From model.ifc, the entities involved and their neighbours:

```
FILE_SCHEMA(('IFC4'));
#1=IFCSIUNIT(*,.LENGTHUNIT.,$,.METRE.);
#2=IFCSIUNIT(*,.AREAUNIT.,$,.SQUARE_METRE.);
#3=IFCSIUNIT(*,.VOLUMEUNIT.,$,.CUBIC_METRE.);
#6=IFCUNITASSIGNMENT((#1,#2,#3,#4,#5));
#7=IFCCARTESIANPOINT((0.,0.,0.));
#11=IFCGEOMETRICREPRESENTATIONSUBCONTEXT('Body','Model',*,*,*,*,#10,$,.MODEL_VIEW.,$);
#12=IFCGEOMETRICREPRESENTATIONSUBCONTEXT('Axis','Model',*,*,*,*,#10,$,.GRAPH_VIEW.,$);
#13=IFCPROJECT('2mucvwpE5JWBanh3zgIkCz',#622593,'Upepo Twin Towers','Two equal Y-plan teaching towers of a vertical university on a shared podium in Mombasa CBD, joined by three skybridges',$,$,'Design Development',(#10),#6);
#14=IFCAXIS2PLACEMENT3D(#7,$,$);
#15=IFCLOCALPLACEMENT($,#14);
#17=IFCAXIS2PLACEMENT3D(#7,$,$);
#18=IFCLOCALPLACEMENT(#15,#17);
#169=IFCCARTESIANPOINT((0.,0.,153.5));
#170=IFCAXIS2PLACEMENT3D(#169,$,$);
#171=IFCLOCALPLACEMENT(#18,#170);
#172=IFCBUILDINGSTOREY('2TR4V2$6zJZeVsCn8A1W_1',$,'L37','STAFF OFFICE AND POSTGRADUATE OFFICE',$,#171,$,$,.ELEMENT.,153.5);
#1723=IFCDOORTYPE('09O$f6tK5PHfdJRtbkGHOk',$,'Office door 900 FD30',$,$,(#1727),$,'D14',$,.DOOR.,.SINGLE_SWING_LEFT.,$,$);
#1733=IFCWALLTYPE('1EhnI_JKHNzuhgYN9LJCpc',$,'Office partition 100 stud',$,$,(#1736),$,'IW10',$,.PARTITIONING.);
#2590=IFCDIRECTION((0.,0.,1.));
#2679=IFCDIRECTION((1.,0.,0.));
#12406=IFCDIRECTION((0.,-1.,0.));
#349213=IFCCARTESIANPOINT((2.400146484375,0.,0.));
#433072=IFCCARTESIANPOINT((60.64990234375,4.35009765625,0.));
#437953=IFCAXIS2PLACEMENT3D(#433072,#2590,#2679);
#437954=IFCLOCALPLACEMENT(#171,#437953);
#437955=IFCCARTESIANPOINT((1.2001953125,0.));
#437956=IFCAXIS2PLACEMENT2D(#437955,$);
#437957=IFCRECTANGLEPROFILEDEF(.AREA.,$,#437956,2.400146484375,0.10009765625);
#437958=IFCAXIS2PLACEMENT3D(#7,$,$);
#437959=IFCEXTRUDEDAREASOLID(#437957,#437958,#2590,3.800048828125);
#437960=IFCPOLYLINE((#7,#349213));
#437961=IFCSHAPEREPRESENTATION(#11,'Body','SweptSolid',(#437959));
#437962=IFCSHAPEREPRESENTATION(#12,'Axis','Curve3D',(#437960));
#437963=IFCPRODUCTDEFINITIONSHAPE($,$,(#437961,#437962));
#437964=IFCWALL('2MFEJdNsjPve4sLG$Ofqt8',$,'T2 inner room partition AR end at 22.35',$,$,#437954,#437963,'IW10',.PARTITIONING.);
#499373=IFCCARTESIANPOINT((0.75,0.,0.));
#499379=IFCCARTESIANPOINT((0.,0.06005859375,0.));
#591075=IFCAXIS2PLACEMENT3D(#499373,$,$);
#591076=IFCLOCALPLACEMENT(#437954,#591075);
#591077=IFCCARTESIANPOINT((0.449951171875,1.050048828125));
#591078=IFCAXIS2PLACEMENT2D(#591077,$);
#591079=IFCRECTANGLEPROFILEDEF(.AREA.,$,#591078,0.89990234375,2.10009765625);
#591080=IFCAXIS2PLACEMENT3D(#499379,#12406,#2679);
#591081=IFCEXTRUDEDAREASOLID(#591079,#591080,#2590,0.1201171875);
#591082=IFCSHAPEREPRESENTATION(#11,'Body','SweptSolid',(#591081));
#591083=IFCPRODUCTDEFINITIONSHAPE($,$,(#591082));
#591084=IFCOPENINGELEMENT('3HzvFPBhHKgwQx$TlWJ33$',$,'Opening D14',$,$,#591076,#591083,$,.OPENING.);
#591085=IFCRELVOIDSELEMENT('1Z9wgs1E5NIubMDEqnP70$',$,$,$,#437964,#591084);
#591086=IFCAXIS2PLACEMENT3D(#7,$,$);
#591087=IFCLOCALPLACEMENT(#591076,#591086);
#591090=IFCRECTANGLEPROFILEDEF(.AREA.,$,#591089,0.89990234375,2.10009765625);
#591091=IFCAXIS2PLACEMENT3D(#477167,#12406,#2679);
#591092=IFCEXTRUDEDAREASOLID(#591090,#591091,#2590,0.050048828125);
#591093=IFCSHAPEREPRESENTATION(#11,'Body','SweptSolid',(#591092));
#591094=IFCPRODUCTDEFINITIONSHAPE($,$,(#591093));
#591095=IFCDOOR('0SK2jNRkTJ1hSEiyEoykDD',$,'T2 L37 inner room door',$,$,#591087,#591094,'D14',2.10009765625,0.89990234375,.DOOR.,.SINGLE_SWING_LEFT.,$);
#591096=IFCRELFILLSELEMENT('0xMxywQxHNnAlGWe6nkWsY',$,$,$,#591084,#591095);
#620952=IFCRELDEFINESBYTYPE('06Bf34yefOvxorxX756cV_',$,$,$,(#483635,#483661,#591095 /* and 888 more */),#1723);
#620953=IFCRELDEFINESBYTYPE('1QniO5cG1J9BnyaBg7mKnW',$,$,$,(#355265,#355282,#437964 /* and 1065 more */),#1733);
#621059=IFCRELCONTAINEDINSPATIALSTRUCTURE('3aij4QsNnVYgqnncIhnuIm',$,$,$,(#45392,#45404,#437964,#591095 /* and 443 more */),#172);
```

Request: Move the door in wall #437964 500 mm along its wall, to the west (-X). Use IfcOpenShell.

```python
import ifcopenshell
import ifcopenshell.api.geometry
import ifcopenshell.util.placement
import ifcopenshell.util.unit

model = ifcopenshell.open("model.ifc")
unit_scale = ifcopenshell.util.unit.calculate_unit_scale(model)

door = model.by_guid("0SK2jNRkTJ1hSEiyEoykDD")
opening = door.FillsVoids[0].RelatingOpeningElement
wall = opening.VoidsElements[0].RelatingBuildingElement

wall_matrix = ifcopenshell.util.placement.get_local_placement(wall.ObjectPlacement)
shift = wall_matrix[:3, 0] * -0.5 / unit_scale
before = ifcopenshell.util.placement.get_local_placement(door.ObjectPlacement)[:3, 3].copy()

# The door is placed relative to its opening, so it follows when the opening moves.
matrix = ifcopenshell.util.placement.get_local_placement(opening.ObjectPlacement)
matrix[:3, 3] += shift
ifcopenshell.api.geometry.edit_object_placement(
    model, product=opening, matrix=matrix, is_si=False, should_transform_children=True
)

after = ifcopenshell.util.placement.get_local_placement(door.ObjectPlacement)[:3, 3]
print("door moved by", (after - before).round(3) + 0.0)

model.write("model_edited.ifc")
```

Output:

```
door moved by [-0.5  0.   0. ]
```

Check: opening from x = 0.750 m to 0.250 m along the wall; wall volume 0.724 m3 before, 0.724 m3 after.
